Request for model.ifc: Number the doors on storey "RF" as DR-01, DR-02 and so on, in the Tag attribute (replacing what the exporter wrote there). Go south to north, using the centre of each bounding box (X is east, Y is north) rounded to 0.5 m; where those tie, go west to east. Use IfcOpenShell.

First a look at what the model holds.

```python
import ifcopenshell
import ifcopenshell.util.element
import ifcopenshell.util.placement

model = ifcopenshell.open("model.ifc")
print(model.schema)
storey = next(s for s in model.by_type("IfcBuildingStorey") if s.Name == "RF")
doors = [e for e in ifcopenshell.util.element.get_decomposition(storey) if e.is_a("IfcDoor")]
for e in sorted(doors, key=lambda e: e.id()):
    origin = ifcopenshell.util.placement.get_local_placement(e.ObjectPlacement)[:3, 3]
    print(e.id(), e.Tag, e.Name, origin.round(2) + 0.0, sep=" | ")
```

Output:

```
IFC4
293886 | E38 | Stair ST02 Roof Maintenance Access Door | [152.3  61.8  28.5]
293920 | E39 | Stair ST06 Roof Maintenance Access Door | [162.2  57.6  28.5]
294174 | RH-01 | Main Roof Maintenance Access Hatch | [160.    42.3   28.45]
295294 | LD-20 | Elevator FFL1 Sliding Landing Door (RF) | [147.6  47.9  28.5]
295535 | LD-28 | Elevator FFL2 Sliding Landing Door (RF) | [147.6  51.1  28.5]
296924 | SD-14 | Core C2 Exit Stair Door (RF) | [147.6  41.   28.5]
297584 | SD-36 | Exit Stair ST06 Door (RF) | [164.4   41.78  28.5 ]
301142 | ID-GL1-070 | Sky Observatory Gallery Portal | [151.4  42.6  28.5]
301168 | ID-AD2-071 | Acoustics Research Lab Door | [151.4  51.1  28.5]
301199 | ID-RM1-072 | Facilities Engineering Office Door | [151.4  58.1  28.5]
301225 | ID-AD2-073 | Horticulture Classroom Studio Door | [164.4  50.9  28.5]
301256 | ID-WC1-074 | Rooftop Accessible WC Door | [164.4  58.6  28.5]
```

```python
import ifcopenshell
import ifcopenshell.geom
import ifcopenshell.util.element
import ifcopenshell.util.shape

model = ifcopenshell.open("model.ifc")
settings = ifcopenshell.geom.settings()
settings.set("use-world-coords", True)


def centre(element):
    shape = ifcopenshell.geom.create_shape(settings, element)
    return ifcopenshell.util.shape.get_bbox_centroid(shape.geometry)


storey = next(s for s in model.by_type("IfcBuildingStorey") if s.Name == "RF")
doors = [e for e in ifcopenshell.util.element.get_decomposition(storey) if e.is_a("IfcDoor")]

# Insertion points can sit at a corner or the storey origin, so sort by the geometry (in metres).
centres = {e: centre(e) for e in doors}
doors.sort(key=lambda e: (round(centres[e][1] / 0.5), centres[e][0]))

for i, e in enumerate(doors, start=1):
    number = f"DR-{i:02d}"
    e.Tag = number
    print(e.id(), number)

model.write("model_updated.ifc")
```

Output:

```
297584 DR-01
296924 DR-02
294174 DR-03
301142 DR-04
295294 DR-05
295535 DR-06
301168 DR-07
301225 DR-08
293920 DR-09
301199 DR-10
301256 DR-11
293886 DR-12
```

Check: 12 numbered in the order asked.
